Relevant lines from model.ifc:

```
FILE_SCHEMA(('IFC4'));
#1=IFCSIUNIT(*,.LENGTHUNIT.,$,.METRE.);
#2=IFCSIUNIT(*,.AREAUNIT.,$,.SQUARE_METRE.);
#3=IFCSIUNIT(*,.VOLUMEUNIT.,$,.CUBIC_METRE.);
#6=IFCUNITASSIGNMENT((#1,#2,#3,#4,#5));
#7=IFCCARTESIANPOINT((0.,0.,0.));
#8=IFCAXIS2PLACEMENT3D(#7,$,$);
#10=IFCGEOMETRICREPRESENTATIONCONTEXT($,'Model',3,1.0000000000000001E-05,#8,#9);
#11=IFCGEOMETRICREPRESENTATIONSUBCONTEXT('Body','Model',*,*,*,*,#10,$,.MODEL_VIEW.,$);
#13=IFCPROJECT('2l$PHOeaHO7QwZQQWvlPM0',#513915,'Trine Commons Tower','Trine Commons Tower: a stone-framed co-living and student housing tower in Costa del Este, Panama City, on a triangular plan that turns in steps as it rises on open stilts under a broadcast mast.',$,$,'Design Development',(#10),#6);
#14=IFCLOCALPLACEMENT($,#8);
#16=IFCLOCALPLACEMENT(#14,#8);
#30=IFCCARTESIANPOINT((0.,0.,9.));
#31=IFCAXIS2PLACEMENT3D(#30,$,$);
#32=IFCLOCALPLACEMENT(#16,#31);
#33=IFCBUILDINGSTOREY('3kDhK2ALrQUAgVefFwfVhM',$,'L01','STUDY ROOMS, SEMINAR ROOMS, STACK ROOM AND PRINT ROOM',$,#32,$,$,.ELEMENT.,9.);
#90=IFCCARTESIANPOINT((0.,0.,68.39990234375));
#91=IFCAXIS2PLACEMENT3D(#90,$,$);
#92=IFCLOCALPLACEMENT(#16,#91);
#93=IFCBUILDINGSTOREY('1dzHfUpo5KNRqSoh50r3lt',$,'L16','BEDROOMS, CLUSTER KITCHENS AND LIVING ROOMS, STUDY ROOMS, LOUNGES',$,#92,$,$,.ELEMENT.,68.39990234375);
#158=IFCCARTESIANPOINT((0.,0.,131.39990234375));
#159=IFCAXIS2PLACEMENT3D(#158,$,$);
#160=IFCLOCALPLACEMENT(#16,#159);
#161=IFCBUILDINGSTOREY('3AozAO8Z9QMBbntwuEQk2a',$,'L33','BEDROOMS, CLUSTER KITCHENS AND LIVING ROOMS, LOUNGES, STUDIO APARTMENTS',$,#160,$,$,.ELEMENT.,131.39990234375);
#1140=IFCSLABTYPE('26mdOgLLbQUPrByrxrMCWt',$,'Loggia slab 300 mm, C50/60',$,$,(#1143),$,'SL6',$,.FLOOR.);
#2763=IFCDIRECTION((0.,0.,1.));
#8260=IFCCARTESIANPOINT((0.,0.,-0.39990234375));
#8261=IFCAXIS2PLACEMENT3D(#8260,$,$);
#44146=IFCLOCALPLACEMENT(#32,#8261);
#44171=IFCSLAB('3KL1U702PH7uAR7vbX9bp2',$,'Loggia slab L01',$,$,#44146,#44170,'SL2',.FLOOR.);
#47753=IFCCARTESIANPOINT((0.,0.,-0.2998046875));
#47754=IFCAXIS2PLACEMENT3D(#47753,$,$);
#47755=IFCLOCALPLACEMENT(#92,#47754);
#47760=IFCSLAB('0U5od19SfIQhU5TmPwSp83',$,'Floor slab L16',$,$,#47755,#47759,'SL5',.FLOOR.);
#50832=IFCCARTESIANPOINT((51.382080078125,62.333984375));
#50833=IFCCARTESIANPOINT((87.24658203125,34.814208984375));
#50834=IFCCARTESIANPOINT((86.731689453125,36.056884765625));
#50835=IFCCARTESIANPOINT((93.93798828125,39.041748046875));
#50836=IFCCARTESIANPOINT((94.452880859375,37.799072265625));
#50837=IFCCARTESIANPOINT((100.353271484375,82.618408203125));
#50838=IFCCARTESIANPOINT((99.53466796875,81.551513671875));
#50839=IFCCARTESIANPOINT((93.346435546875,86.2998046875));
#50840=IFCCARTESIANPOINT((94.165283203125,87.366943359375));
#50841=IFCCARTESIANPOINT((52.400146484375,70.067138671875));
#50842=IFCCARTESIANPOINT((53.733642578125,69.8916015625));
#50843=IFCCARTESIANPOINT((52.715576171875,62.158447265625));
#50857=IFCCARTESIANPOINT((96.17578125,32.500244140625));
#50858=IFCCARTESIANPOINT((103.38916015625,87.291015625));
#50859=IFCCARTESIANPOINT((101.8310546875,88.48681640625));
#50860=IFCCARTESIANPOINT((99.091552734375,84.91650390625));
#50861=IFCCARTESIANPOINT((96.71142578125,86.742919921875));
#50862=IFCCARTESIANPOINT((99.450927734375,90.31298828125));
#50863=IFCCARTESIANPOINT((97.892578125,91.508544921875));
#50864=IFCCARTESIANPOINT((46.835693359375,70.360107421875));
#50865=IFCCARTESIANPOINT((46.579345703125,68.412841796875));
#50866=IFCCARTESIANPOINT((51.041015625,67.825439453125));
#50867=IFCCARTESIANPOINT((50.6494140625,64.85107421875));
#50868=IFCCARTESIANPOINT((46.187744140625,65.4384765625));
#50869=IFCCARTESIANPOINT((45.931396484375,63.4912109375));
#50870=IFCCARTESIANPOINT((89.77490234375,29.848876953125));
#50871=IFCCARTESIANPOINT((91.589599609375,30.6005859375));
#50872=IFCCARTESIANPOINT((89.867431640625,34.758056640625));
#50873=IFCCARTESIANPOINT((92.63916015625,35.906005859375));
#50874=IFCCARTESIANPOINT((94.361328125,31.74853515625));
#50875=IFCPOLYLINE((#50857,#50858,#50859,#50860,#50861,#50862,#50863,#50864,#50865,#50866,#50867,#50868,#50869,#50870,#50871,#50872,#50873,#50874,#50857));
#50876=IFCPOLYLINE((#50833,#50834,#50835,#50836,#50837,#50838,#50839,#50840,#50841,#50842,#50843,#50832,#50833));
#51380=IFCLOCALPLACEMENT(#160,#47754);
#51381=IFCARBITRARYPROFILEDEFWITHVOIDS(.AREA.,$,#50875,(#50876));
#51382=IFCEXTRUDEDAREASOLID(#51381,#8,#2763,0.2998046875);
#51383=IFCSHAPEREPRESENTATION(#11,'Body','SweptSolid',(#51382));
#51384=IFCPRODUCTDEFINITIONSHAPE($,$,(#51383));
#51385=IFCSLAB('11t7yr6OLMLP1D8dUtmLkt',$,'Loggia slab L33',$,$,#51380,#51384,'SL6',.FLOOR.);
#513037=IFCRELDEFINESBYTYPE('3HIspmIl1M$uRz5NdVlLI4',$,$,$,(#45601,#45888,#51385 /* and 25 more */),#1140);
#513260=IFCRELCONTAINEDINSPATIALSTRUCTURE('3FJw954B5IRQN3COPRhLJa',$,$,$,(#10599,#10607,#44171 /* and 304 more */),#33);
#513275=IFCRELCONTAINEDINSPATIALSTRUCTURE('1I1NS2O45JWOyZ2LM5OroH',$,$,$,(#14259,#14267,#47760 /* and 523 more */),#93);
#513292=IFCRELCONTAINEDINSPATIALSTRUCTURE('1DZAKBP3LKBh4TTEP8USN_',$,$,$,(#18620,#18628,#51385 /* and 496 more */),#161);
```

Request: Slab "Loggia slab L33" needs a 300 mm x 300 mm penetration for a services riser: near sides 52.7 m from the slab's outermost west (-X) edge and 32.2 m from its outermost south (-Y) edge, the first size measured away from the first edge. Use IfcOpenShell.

```python
import numpy as np
import ifcopenshell
import ifcopenshell.api.feature
import ifcopenshell.api.geometry
import ifcopenshell.api.root
import ifcopenshell.geom
import ifcopenshell.util.placement
import ifcopenshell.util.representation
import ifcopenshell.util.shape
import ifcopenshell.util.unit

model = ifcopenshell.open("model.ifc")
unit_scale = ifcopenshell.util.unit.calculate_unit_scale(model)
settings = ifcopenshell.geom.settings()


def volume(element):
    """Net volume in cubic metres, openings subtracted."""
    shape = ifcopenshell.geom.create_shape(settings, element)
    return ifcopenshell.util.shape.get_volume(shape.geometry)


slab = model.by_guid("11t7yr6OLMLP1D8dUtmLkt")
before = volume(slab)

# Extent in the slab's own axes, in metres. The edges named are its -X and -Y sides.
slab_shape = ifcopenshell.geom.create_shape(settings, slab)
vertices = ifcopenshell.util.shape.get_vertices(slab_shape.geometry)
x_min, y_min, bottom = vertices.min(axis=0)
top = vertices[:, 2].max()

opening = ifcopenshell.api.root.create_entity(model, ifc_class="IfcOpeningElement", name="Services riser opening", predefined_type="OPENING")
context = ifcopenshell.util.representation.get_context(model, "Model", "Body", "MODEL_VIEW")
width, depth = 0.3, 0.3
outline = [(0.0, 0.0), (width, 0.0), (width, depth), (0.0, depth), (0.0, 0.0)]
# Overshoot both faces by 50 mm so the cut is clean.
shape = ifcopenshell.api.geometry.add_slab_representation(
    model, context=context, depth=top - bottom + 0.1, polyline=outline
)
ifcopenshell.api.geometry.assign_representation(model, product=opening, representation=shape)

matrix = ifcopenshell.util.placement.get_local_placement(slab.ObjectPlacement)
matrix[:, 3] = matrix @ np.append(np.array([x_min + 52.7, y_min + 32.2, bottom - 0.05]) / unit_scale, 1.0)
ifcopenshell.api.geometry.edit_object_placement(model, product=opening, matrix=matrix, is_si=False)
ifcopenshell.api.feature.add_feature(model, feature=opening, element=slab)

after = volume(slab)

print(f"slab volume {before:.3f} -> {after:.3f} m3")

model.write("model_rev.ifc")
```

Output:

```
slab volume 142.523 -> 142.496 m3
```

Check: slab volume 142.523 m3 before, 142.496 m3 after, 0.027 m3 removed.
